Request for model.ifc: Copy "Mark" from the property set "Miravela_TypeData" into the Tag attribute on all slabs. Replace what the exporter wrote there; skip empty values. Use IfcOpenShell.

First a look at what the model holds.

```python
import ifcopenshell
import ifcopenshell.util.element

model = ifcopenshell.open("model.ifc")
print(model.schema)
slabs = model.by_type("IfcSlab")
print(len(slabs), "slabs")
for e in slabs[:8]:
    source = ifcopenshell.util.element.get_pset(e, "Miravela_TypeData", "Mark")
    target = e.Tag
    print(e.id(), repr(source), repr(target), sep=" | ")
```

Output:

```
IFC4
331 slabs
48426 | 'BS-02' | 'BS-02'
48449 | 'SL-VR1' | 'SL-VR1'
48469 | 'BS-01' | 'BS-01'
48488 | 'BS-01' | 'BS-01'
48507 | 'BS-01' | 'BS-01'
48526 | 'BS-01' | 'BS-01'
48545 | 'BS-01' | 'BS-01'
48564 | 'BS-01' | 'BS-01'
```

```python
import ifcopenshell
import ifcopenshell.util.element

model = ifcopenshell.open("model.ifc")

count = 0
for e in model.by_type("IfcSlab"):
    value = ifcopenshell.util.element.get_pset(e, "Miravela_TypeData", "Mark")
    current = e.Tag
    if not value or not value.strip() or current == value:
        continue
    e.Tag = value
    count += 1

print(count, "slabs updated")

model.write("model_updated.ifc")
```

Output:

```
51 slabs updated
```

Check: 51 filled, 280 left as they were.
